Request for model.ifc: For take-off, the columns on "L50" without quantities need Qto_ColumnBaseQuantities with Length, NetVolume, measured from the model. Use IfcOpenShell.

First a look at what the model holds.

```python
import ifcopenshell
import ifcopenshell.util.element
import ifcopenshell.util.unit

model = ifcopenshell.open("model.ifc")
print(model.schema)
for unit_type in ("LENGTHUNIT", "AREAUNIT", "VOLUMEUNIT"):
    print(unit_type, ifcopenshell.util.unit.calculate_unit_scale(model, unit_type))
storey = next(s for s in model.by_type("IfcBuildingStorey") if s.Name == "L50")
columns = [e for e in ifcopenshell.util.element.get_decomposition(storey) if e.is_a("IfcColumn")]
for e in sorted(columns, key=lambda e: e.id()):
    print(e.id(), e.is_a(), e.Name, list(ifcopenshell.util.element.get_psets(e, qtos_only=True)), sep=" | ")
```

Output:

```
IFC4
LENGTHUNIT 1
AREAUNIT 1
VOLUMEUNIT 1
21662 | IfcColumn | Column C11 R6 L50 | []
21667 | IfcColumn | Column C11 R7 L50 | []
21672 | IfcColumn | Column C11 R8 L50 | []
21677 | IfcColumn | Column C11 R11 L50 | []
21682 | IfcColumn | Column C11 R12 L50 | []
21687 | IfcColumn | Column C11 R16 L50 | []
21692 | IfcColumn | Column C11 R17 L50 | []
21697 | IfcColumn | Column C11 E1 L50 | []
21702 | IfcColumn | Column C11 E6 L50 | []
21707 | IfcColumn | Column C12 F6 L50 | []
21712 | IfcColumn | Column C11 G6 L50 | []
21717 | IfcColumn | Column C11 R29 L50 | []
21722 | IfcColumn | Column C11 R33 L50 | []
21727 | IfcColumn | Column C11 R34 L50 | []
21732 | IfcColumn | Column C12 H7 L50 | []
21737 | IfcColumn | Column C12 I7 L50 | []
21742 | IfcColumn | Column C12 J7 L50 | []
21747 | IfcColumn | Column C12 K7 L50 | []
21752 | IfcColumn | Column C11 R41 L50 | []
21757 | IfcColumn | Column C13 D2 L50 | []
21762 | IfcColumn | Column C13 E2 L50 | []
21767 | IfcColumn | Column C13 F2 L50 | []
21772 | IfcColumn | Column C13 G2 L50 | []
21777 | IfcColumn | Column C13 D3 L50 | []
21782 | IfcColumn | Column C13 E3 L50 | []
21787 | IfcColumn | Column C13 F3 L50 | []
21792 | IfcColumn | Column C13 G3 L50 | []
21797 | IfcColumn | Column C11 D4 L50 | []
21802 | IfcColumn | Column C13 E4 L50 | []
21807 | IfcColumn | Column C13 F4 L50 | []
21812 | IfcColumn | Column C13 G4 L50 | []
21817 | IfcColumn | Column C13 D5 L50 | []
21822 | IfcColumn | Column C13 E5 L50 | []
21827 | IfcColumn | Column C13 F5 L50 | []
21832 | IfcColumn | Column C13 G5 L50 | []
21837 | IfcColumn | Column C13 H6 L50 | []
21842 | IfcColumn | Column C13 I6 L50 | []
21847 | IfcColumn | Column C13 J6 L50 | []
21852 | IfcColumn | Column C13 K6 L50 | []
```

```python
import ifcopenshell
import ifcopenshell.api.pset
import ifcopenshell.geom
import ifcopenshell.util.element
import ifcopenshell.util.shape
import ifcopenshell.util.unit

model = ifcopenshell.open("model.ifc")
unit_scale = ifcopenshell.util.unit.calculate_unit_scale(model)
volume_scale = ifcopenshell.util.unit.calculate_unit_scale(model, "VOLUMEUNIT")
settings = ifcopenshell.geom.settings()

storey = next(s for s in model.by_type("IfcBuildingStorey") if s.Name == "L50")
columns = [e for e in ifcopenshell.util.element.get_decomposition(storey) if e.is_a("IfcColumn")]

for e in sorted(columns, key=lambda e: e.id()):
    if ifcopenshell.util.element.get_psets(e, qtos_only=True, should_inherit=False):
        continue
    # Geometry comes back in metres, in the element's own axes.
    shape = ifcopenshell.geom.create_shape(settings, e)
    values = {
        "Length": ifcopenshell.util.shape.get_z(shape.geometry) / unit_scale,
        "NetVolume": ifcopenshell.util.shape.get_volume(shape.geometry) / volume_scale,
    }
    qto = ifcopenshell.api.pset.add_qto(model, product=e, name="Qto_ColumnBaseQuantities")
    ifcopenshell.api.pset.edit_qto(model, qto=qto, properties=values)
    print(e.id(), {k: round(v, 3) for k, v in values.items()})

model.write("model_updated.ifc")
```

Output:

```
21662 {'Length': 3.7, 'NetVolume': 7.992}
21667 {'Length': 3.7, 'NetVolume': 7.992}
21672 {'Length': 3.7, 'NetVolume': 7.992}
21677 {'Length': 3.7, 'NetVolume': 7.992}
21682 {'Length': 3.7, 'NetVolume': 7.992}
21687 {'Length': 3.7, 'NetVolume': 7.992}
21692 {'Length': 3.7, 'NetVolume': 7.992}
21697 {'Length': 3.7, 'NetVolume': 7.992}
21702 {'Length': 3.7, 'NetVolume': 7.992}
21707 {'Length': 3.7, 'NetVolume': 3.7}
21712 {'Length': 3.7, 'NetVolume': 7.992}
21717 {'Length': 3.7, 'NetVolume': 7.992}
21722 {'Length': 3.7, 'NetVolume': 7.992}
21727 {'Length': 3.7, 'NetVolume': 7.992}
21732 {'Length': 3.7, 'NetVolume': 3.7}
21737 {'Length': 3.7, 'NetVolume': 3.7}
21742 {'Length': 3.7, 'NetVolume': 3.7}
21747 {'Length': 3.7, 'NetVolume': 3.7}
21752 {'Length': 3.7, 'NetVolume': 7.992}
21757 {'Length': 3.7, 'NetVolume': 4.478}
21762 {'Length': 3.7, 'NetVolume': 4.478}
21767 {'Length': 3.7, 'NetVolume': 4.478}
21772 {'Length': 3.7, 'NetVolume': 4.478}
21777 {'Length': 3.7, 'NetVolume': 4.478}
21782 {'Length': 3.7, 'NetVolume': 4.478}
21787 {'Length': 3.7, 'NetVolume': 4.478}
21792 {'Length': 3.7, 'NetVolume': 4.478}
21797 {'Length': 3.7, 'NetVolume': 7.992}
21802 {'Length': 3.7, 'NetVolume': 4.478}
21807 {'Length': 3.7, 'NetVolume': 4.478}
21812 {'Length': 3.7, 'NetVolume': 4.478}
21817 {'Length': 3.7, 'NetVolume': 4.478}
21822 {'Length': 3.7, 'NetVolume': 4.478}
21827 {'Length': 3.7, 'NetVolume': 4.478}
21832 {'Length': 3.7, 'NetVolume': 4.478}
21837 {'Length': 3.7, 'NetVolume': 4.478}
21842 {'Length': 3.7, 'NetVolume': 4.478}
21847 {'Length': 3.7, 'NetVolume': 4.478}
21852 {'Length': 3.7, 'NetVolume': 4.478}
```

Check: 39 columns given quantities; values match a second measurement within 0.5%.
